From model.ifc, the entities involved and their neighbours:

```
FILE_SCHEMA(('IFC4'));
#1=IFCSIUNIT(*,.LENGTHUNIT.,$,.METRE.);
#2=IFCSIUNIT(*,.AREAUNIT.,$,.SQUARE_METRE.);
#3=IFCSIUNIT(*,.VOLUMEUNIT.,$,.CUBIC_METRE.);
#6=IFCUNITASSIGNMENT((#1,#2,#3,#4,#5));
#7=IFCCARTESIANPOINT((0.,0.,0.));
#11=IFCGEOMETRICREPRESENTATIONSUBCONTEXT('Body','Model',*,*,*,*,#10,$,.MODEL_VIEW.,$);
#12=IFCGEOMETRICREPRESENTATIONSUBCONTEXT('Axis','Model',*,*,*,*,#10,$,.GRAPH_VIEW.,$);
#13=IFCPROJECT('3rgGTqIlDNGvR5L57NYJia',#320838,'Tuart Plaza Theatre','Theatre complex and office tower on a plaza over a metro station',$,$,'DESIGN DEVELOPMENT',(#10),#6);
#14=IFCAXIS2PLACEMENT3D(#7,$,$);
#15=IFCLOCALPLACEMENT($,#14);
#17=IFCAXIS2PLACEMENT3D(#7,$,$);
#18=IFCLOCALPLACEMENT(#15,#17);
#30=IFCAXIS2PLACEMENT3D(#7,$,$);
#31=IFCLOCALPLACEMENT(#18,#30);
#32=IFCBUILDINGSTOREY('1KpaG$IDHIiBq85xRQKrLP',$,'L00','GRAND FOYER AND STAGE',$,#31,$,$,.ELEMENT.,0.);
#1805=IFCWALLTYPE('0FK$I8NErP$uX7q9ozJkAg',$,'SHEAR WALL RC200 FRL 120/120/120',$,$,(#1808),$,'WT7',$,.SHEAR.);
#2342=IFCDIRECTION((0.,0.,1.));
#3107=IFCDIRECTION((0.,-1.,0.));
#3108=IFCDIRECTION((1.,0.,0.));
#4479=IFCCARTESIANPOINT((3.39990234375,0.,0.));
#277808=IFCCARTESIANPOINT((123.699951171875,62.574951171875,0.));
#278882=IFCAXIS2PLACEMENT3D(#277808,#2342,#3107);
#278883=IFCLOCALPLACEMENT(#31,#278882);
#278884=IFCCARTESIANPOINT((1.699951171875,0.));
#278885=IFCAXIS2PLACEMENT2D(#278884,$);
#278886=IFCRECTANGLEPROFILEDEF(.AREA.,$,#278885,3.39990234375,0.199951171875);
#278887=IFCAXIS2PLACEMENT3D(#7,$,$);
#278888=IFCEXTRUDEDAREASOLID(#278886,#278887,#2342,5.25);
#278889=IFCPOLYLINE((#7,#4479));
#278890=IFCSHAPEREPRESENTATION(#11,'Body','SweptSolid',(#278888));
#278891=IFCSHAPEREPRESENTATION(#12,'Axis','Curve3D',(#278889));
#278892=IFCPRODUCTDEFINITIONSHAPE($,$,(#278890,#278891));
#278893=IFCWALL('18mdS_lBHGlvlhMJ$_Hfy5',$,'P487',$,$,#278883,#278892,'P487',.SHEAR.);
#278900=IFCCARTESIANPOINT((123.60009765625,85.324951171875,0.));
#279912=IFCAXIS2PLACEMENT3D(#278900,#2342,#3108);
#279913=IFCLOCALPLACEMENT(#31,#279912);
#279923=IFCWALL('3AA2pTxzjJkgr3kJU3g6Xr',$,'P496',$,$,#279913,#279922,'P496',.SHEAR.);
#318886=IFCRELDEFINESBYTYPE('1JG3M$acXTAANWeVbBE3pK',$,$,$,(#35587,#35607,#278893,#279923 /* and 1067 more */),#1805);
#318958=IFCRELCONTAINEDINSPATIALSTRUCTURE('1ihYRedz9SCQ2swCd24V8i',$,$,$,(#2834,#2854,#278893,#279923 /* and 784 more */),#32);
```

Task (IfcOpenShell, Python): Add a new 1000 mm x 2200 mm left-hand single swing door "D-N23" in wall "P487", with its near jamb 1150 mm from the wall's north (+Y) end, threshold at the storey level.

```python
import numpy as np
import ifcopenshell
import ifcopenshell.api.feature
import ifcopenshell.api.geometry
import ifcopenshell.api.root
import ifcopenshell.api.spatial
import ifcopenshell.geom
import ifcopenshell.util.element
import ifcopenshell.util.placement
import ifcopenshell.util.representation
import ifcopenshell.util.shape
import ifcopenshell.util.unit

model = ifcopenshell.open("model.ifc")
unit_scale = ifcopenshell.util.unit.calculate_unit_scale(model)
settings = ifcopenshell.geom.settings()


def volume(element):
    """Net volume in cubic metres, openings subtracted."""
    shape = ifcopenshell.geom.create_shape(settings, element)
    return ifcopenshell.util.shape.get_volume(shape.geometry)


wall = model.by_guid("18mdS_lBHGlvlhMJ$_Hfy5")
storey = ifcopenshell.util.element.get_container(wall, ifc_class="IfcBuildingStorey")
context = ifcopenshell.util.representation.get_context(model, "Model", "Body", "MODEL_VIEW")
before = volume(wall)

width, height, from_end, sill = 1, 2.2, 1.15, 0.0  # metres

# The wall runs along its own X axis, and the end named is its -X end.
wall_shape = ifcopenshell.geom.create_shape(settings, wall)
x, y, z = ifcopenshell.util.shape.get_vertices(wall_shape.geometry).T
start = x.min() + from_end
face, thickness = float(y.min()), float(y.max() - y.min())
wall_matrix = ifcopenshell.util.placement.get_local_placement(wall.ObjectPlacement)
level = ifcopenshell.util.placement.get_local_placement(storey.ObjectPlacement)[2, 3]


def in_wall(x, y):
    """Placement at x, y metres in the wall's axes, at sill height."""
    matrix = wall_matrix.copy()
    matrix[:, 3] = wall_matrix @ np.array([x / unit_scale, y / unit_scale, 0.0, 1.0])
    matrix[2, 3] = level + sill / unit_scale
    return matrix


# Opening: a box that overshoots both wall faces by 50 mm.
opening = ifcopenshell.api.root.create_entity(model, ifc_class="IfcOpeningElement", predefined_type="OPENING")
box = ifcopenshell.api.geometry.add_wall_representation(
    model, context=context, length=width, height=height, thickness=thickness + 0.1
)
ifcopenshell.api.geometry.assign_representation(model, product=opening, representation=box)
ifcopenshell.api.geometry.edit_object_placement(model, product=opening, matrix=in_wall(start, face - 0.05), is_si=False)
ifcopenshell.api.feature.add_feature(model, feature=opening, element=wall)

door = ifcopenshell.api.root.create_entity(model, ifc_class="IfcDoor", name="D-N23", predefined_type="DOOR")
door.OverallWidth, door.OverallHeight = width / unit_scale, height / unit_scale
door.OperationType = "SINGLE_SWING_LEFT"
body = ifcopenshell.api.geometry.add_door_representation(
    model,
    context=context,
    overall_width=door.OverallWidth,
    overall_height=door.OverallHeight,
    operation_type="SINGLE_SWING_LEFT",
    lining_properties={"LiningDepth": thickness / unit_scale, "ThresholdDepth": thickness / unit_scale},
)
ifcopenshell.api.geometry.assign_representation(model, product=door, representation=body)
ifcopenshell.api.spatial.assign_container(model, products=[door], relating_structure=storey)
ifcopenshell.api.feature.add_filling(model, opening=opening, element=door)

# The lining spans the wall, so the door starts at the wall face.
ifcopenshell.api.geometry.edit_object_placement(model, product=door, matrix=in_wall(start, face), is_si=False)

after = volume(wall)

print(f"wall volume {before:.3f} -> {after:.3f} m3")

model.write("model-out.ifc")
```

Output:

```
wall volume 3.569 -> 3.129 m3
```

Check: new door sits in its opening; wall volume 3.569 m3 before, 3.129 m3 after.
